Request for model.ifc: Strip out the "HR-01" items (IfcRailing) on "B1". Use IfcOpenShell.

First a look at what the model holds.

```python
import ifcopenshell
import ifcopenshell.util.element

model = ifcopenshell.open("model.ifc")
print(model.schema)
storey = next(s for s in model.by_type("IfcBuildingStorey") if s.Name == "B1")
railings = [e for e in ifcopenshell.util.element.get_decomposition(storey) if e.is_a("IfcRailing")]
seen = {}
for e in railings:
    element_type = ifcopenshell.util.element.get_type(e)
    name = element_type.Name if element_type not in (None, e) else None
    seen[name] = seen.get(name, 0) + 1
for name, count in sorted(seen.items(), key=str):
    print(count, "x", name)
```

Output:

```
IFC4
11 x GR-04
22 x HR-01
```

```python
import ifcopenshell
import ifcopenshell.api.root
import ifcopenshell.util.element

model = ifcopenshell.open("model.ifc")

storey = next(s for s in model.by_type("IfcBuildingStorey") if s.Name == "B1")
railings = [e for e in ifcopenshell.util.element.get_decomposition(storey) if e.is_a("IfcRailing")]
targets = [e for e in railings if (t := ifcopenshell.util.element.get_type(e)) not in (None, e) and t.Name == "HR-01"]

for e in targets:
    ifcopenshell.api.root.remove_product(model, product=e)
print(len(targets), "removed")

model.write("model_v2.ifc")
```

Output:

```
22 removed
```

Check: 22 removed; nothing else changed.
